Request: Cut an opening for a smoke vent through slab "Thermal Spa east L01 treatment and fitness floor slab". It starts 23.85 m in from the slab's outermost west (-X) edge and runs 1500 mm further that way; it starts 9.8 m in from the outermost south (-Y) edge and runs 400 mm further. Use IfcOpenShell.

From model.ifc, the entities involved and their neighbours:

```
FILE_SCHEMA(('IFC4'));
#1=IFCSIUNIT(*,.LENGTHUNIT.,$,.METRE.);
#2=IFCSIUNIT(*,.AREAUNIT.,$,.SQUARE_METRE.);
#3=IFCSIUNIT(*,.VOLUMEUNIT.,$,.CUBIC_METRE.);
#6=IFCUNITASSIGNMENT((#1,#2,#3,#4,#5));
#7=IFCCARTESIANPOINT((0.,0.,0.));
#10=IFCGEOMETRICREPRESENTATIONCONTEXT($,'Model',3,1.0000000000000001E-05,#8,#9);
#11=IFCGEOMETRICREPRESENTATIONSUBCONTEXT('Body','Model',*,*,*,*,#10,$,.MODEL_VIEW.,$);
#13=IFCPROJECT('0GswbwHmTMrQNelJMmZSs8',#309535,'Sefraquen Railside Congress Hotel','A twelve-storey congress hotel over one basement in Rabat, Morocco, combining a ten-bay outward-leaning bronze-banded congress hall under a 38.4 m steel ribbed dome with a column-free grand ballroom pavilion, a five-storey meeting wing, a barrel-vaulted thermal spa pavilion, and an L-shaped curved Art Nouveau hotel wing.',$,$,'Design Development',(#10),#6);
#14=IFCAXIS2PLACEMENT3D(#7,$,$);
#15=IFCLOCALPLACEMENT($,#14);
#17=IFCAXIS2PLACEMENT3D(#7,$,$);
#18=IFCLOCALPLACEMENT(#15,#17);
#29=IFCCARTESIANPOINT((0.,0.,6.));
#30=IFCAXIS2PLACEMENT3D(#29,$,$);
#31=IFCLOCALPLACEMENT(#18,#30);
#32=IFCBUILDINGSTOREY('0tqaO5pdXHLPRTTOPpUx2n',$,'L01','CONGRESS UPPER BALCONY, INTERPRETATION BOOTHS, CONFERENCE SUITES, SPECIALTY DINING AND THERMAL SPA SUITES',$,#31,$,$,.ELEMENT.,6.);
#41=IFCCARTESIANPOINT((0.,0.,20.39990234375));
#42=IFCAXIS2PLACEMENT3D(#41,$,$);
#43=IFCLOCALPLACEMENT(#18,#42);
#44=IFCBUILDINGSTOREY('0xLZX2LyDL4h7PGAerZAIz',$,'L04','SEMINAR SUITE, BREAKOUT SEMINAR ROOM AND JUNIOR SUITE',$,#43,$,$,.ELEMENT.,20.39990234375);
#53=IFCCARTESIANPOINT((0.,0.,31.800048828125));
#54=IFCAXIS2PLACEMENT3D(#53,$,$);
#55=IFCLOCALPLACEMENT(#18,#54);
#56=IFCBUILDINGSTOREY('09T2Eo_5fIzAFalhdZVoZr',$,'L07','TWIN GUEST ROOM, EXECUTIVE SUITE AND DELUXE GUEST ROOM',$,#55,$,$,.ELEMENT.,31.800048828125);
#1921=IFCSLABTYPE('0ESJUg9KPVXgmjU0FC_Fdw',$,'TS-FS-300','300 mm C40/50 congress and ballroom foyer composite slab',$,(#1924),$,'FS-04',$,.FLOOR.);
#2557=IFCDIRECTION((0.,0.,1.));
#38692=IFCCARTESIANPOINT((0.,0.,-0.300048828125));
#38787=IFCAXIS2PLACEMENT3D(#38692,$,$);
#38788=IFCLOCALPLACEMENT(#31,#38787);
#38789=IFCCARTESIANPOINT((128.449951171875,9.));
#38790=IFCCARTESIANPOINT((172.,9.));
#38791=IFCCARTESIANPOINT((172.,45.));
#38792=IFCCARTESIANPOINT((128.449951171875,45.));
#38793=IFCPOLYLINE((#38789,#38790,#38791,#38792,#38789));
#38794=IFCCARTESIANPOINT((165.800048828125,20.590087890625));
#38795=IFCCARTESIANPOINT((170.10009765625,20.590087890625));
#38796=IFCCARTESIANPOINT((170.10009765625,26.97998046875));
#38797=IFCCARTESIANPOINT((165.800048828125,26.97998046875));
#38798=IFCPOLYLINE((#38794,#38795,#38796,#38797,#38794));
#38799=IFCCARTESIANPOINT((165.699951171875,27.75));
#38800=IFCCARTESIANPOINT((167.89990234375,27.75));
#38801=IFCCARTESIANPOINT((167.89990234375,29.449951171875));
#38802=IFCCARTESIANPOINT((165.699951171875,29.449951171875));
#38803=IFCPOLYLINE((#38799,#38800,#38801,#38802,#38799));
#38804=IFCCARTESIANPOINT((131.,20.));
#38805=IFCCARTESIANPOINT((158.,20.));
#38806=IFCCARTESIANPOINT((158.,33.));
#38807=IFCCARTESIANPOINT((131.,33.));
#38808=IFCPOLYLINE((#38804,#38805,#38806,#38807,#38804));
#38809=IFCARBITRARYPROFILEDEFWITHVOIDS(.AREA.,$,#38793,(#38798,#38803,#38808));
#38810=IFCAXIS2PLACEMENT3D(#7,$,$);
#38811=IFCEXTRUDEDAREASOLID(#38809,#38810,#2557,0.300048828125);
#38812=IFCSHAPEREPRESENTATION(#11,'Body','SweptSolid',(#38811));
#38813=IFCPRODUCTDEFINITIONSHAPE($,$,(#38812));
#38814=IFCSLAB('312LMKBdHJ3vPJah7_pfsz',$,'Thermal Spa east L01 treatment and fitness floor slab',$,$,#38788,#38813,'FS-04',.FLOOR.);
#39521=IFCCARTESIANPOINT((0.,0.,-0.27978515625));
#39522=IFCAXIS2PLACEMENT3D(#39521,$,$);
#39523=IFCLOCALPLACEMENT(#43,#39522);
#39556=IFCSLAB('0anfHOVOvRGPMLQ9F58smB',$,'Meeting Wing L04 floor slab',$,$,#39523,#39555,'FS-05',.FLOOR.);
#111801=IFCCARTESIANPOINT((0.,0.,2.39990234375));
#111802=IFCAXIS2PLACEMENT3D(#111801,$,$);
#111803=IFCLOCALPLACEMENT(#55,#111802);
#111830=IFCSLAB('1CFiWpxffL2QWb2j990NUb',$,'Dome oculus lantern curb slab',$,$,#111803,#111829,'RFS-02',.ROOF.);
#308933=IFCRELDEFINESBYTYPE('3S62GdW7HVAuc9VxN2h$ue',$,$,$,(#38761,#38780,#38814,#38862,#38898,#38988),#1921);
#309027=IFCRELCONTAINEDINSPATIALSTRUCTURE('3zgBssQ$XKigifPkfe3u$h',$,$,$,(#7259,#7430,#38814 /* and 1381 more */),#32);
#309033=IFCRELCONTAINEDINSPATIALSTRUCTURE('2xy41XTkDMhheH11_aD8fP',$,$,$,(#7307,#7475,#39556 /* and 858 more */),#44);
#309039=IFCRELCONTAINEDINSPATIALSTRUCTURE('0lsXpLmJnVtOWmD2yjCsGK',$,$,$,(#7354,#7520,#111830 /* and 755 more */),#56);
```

```python
import numpy as np
import ifcopenshell
import ifcopenshell.api.feature
import ifcopenshell.api.geometry
import ifcopenshell.api.root
import ifcopenshell.geom
import ifcopenshell.util.placement
import ifcopenshell.util.representation
import ifcopenshell.util.shape
import ifcopenshell.util.unit

model = ifcopenshell.open("model.ifc")
unit_scale = ifcopenshell.util.unit.calculate_unit_scale(model)
settings = ifcopenshell.geom.settings()


def volume(element):
    """Net volume in cubic metres, openings subtracted."""
    shape = ifcopenshell.geom.create_shape(settings, element)
    return ifcopenshell.util.shape.get_volume(shape.geometry)


slab = model.by_guid("312LMKBdHJ3vPJah7_pfsz")
before = volume(slab)

# Extent in the slab's own axes, in metres. The edges named are its -X and -Y sides.
slab_shape = ifcopenshell.geom.create_shape(settings, slab)
vertices = ifcopenshell.util.shape.get_vertices(slab_shape.geometry)
x_min, y_min, bottom = vertices.min(axis=0)
top = vertices[:, 2].max()

opening = ifcopenshell.api.root.create_entity(model, ifc_class="IfcOpeningElement", name="Smoke vent opening", predefined_type="OPENING")
context = ifcopenshell.util.representation.get_context(model, "Model", "Body", "MODEL_VIEW")
width, depth = 1.5, 0.4
outline = [(0.0, 0.0), (width, 0.0), (width, depth), (0.0, depth), (0.0, 0.0)]
# Overshoot both faces by 50 mm so the cut is clean.
shape = ifcopenshell.api.geometry.add_slab_representation(
    model, context=context, depth=top - bottom + 0.1, polyline=outline
)
ifcopenshell.api.geometry.assign_representation(model, product=opening, representation=shape)

matrix = ifcopenshell.util.placement.get_local_placement(slab.ObjectPlacement)
matrix[:, 3] = matrix @ np.append(np.array([x_min + 23.85, y_min + 9.8, bottom - 0.05]) / unit_scale, 1.0)
ifcopenshell.api.geometry.edit_object_placement(model, product=opening, matrix=matrix, is_si=False)
ifcopenshell.api.feature.add_feature(model, feature=opening, element=slab)

after = volume(slab)

print(f"slab volume {before:.3f} -> {after:.3f} m3")

model.write("model_v2.ifc")
```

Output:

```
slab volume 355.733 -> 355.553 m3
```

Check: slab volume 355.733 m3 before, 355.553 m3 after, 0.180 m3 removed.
